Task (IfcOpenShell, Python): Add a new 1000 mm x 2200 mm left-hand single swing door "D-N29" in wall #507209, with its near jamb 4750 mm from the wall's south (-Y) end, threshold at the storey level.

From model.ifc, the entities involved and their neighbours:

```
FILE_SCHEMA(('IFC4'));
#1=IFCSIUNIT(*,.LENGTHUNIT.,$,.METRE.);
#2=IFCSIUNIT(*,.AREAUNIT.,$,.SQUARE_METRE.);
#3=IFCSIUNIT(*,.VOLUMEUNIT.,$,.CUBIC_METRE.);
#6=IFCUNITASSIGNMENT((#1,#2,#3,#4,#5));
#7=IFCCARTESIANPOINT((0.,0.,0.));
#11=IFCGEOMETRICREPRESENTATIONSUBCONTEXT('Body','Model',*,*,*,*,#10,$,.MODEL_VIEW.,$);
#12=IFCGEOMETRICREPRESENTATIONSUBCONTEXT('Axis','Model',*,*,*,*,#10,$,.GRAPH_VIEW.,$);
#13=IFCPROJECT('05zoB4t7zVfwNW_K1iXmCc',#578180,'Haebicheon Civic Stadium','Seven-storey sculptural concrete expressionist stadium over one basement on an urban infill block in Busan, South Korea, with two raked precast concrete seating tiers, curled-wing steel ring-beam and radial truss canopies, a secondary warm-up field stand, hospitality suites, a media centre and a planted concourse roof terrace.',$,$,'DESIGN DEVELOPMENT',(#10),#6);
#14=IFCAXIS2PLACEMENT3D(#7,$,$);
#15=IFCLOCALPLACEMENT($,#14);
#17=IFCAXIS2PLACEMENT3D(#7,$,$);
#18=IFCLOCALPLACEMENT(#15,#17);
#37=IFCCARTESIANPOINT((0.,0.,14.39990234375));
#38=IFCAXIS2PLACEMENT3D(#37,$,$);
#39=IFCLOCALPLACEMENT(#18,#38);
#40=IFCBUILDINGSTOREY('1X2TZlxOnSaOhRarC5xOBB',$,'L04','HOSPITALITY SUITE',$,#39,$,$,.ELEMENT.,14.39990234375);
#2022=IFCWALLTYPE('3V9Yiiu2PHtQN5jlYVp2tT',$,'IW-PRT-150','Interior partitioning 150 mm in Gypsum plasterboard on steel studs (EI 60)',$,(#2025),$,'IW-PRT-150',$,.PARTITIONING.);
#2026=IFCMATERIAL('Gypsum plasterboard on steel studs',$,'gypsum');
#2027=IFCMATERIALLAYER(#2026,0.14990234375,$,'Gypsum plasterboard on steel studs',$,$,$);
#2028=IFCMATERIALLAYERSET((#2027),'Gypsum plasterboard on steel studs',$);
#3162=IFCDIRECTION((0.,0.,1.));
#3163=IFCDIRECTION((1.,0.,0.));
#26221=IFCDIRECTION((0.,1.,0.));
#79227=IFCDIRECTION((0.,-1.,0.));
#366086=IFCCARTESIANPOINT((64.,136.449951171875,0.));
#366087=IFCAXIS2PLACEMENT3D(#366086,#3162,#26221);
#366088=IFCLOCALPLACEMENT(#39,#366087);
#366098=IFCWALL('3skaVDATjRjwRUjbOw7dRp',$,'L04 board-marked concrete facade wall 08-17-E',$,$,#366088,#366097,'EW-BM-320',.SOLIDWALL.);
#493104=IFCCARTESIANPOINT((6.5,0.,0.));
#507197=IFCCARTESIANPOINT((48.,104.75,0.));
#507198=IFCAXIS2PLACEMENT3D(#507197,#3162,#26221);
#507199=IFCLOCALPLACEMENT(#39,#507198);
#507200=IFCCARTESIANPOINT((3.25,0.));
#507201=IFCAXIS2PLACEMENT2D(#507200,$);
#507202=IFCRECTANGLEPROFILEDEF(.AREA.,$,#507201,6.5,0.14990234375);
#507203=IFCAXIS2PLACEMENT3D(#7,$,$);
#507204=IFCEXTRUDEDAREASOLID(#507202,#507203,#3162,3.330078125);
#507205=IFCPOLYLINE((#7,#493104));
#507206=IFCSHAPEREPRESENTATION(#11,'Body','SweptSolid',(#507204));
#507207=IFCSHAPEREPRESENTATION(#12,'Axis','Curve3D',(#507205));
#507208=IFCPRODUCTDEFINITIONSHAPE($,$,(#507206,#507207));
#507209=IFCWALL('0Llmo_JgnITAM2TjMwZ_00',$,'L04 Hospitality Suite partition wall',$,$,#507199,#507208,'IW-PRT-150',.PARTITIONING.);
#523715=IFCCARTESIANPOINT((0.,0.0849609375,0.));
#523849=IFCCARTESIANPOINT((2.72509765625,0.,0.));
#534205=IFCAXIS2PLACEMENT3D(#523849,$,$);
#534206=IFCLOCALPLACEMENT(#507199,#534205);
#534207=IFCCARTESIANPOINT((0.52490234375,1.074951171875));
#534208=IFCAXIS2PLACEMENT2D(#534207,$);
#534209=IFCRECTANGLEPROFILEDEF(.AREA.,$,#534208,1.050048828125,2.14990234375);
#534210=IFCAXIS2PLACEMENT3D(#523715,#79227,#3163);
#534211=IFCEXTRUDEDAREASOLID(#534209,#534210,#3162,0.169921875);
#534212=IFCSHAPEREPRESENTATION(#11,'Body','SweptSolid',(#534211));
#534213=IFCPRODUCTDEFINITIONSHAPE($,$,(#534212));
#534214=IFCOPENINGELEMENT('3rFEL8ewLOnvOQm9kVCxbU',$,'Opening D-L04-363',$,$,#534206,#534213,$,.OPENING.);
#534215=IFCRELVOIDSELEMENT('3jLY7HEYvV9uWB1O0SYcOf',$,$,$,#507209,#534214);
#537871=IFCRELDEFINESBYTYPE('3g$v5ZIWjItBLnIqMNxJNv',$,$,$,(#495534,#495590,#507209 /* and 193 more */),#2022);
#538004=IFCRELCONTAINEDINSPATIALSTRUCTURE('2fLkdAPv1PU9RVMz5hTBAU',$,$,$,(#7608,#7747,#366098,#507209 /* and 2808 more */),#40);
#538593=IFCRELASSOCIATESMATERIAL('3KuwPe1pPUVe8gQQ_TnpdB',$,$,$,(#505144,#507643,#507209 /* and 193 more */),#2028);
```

```python
import numpy as np
import ifcopenshell
import ifcopenshell.api.feature
import ifcopenshell.api.geometry
import ifcopenshell.api.root
import ifcopenshell.api.spatial
import ifcopenshell.geom
import ifcopenshell.util.element
import ifcopenshell.util.placement
import ifcopenshell.util.representation
import ifcopenshell.util.shape
import ifcopenshell.util.unit

model = ifcopenshell.open("model.ifc")
unit_scale = ifcopenshell.util.unit.calculate_unit_scale(model)
settings = ifcopenshell.geom.settings()


def volume(element):
    """Net volume in cubic metres, openings subtracted."""
    shape = ifcopenshell.geom.create_shape(settings, element)
    return ifcopenshell.util.shape.get_volume(shape.geometry)


wall = model.by_id(507209)
storey = ifcopenshell.util.element.get_container(wall, ifc_class="IfcBuildingStorey")
context = ifcopenshell.util.representation.get_context(model, "Model", "Body", "MODEL_VIEW")
before = volume(wall)

width, height, from_end, sill = 1, 2.2, 4.75, 0.0  # metres

# The wall runs along its own X axis, and the end named is its -X end.
wall_shape = ifcopenshell.geom.create_shape(settings, wall)
x, y, z = ifcopenshell.util.shape.get_vertices(wall_shape.geometry).T
start = x.min() + from_end
face, thickness = float(y.min()), float(y.max() - y.min())
wall_matrix = ifcopenshell.util.placement.get_local_placement(wall.ObjectPlacement)
level = ifcopenshell.util.placement.get_local_placement(storey.ObjectPlacement)[2, 3]


def in_wall(x, y):
    """Placement at x, y metres in the wall's axes, at sill height."""
    matrix = wall_matrix.copy()
    matrix[:, 3] = wall_matrix @ np.array([x / unit_scale, y / unit_scale, 0.0, 1.0])
    matrix[2, 3] = level + sill / unit_scale
    return matrix


# Opening: a box that overshoots both wall faces by 50 mm.
opening = ifcopenshell.api.root.create_entity(model, ifc_class="IfcOpeningElement", predefined_type="OPENING")
box = ifcopenshell.api.geometry.add_wall_representation(
    model, context=context, length=width, height=height, thickness=thickness + 0.1
)
ifcopenshell.api.geometry.assign_representation(model, product=opening, representation=box)
ifcopenshell.api.geometry.edit_object_placement(model, product=opening, matrix=in_wall(start, face - 0.05), is_si=False)
ifcopenshell.api.feature.add_feature(model, feature=opening, element=wall)

door = ifcopenshell.api.root.create_entity(model, ifc_class="IfcDoor", name="D-N29", predefined_type="DOOR")
door.OverallWidth, door.OverallHeight = width / unit_scale, height / unit_scale
door.OperationType = "SINGLE_SWING_LEFT"
body = ifcopenshell.api.geometry.add_door_representation(
    model,
    context=context,
    overall_width=door.OverallWidth,
    overall_height=door.OverallHeight,
    operation_type="SINGLE_SWING_LEFT",
    lining_properties={"LiningDepth": thickness / unit_scale, "ThresholdDepth": thickness / unit_scale},
)
ifcopenshell.api.geometry.assign_representation(model, product=door, representation=body)
ifcopenshell.api.spatial.assign_container(model, products=[door], relating_structure=storey)
ifcopenshell.api.feature.add_filling(model, opening=opening, element=door)

# The lining spans the wall, so the door starts at the wall face.
ifcopenshell.api.geometry.edit_object_placement(model, product=door, matrix=in_wall(start, face), is_si=False)

after = volume(wall)

print(f"wall volume {before:.3f} -> {after:.3f} m3")

model.write("model_edited.ifc")
```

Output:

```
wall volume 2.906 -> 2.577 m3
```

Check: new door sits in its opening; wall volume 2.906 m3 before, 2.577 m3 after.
